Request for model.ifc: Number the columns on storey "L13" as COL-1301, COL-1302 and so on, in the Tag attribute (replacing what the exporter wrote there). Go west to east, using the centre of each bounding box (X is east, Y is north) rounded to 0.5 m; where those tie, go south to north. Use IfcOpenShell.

First a look at what the model holds.

```python
import ifcopenshell
import ifcopenshell.util.element
import ifcopenshell.util.placement

model = ifcopenshell.open("model.ifc")
print(model.schema)
storey = next(s for s in model.by_type("IfcBuildingStorey") if s.Name == "L13")
columns = [e for e in ifcopenshell.util.element.get_decomposition(storey) if e.is_a("IfcColumn")]
for e in sorted(columns, key=lambda e: e.id()):
    origin = ifcopenshell.util.placement.get_local_placement(e.ObjectPlacement)[:3, 3]
    print(e.id(), e.Tag, e.Name, origin.round(2) + 0.0, sep=" | ")
```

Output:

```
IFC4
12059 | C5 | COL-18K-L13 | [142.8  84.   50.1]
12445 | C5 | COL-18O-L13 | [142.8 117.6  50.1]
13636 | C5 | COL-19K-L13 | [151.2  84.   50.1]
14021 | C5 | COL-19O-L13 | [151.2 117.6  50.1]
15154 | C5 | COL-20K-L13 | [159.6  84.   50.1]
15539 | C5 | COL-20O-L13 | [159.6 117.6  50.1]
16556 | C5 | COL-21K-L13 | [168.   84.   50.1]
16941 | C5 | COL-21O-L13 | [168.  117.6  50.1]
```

```python
import ifcopenshell
import ifcopenshell.geom
import ifcopenshell.util.element
import ifcopenshell.util.shape

model = ifcopenshell.open("model.ifc")
settings = ifcopenshell.geom.settings()
settings.set("use-world-coords", True)


def centre(element):
    shape = ifcopenshell.geom.create_shape(settings, element)
    return ifcopenshell.util.shape.get_bbox_centroid(shape.geometry)


storey = next(s for s in model.by_type("IfcBuildingStorey") if s.Name == "L13")
columns = [e for e in ifcopenshell.util.element.get_decomposition(storey) if e.is_a("IfcColumn")]

# Insertion points can sit at a corner or the storey origin, so sort by the geometry (in metres).
centres = {e: centre(e) for e in columns}
columns.sort(key=lambda e: (round(centres[e][0] / 0.5), centres[e][1]))

for i, e in enumerate(columns, start=1):
    number = f"COL-13{i:02d}"
    e.Tag = number
    print(e.id(), number)

model.write("model_edited.ifc")
```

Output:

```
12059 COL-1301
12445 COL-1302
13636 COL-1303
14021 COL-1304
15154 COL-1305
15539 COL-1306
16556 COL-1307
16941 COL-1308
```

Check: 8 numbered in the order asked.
